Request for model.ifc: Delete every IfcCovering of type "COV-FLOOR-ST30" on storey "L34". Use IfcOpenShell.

First a look at what the model holds.

```python
import ifcopenshell
import ifcopenshell.util.element

model = ifcopenshell.open("model.ifc")
print(model.schema)
storey = next(s for s in model.by_type("IfcBuildingStorey") if s.Name == "L34")
coverings = [e for e in ifcopenshell.util.element.get_decomposition(storey) if e.is_a("IfcCovering")]
seen = {}
for e in coverings:
    element_type = ifcopenshell.util.element.get_type(e)
    name = element_type.Name if element_type not in (None, e) else None
    seen[name] = seen.get(name, 0) + 1
for name, count in sorted(seen.items(), key=str):
    print(count, "x", name)
```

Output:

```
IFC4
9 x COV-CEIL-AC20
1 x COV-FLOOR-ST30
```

```python
import ifcopenshell
import ifcopenshell.api.root
import ifcopenshell.util.element

model = ifcopenshell.open("model.ifc")

storey = next(s for s in model.by_type("IfcBuildingStorey") if s.Name == "L34")
coverings = [e for e in ifcopenshell.util.element.get_decomposition(storey) if e.is_a("IfcCovering")]
targets = [e for e in coverings if (t := ifcopenshell.util.element.get_type(e)) not in (None, e) and t.Name == "COV-FLOOR-ST30"]

for e in targets:
    ifcopenshell.api.root.remove_product(model, product=e)
print(len(targets), "removed")

model.write("model_edited.ifc")
```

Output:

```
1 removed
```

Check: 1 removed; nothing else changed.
